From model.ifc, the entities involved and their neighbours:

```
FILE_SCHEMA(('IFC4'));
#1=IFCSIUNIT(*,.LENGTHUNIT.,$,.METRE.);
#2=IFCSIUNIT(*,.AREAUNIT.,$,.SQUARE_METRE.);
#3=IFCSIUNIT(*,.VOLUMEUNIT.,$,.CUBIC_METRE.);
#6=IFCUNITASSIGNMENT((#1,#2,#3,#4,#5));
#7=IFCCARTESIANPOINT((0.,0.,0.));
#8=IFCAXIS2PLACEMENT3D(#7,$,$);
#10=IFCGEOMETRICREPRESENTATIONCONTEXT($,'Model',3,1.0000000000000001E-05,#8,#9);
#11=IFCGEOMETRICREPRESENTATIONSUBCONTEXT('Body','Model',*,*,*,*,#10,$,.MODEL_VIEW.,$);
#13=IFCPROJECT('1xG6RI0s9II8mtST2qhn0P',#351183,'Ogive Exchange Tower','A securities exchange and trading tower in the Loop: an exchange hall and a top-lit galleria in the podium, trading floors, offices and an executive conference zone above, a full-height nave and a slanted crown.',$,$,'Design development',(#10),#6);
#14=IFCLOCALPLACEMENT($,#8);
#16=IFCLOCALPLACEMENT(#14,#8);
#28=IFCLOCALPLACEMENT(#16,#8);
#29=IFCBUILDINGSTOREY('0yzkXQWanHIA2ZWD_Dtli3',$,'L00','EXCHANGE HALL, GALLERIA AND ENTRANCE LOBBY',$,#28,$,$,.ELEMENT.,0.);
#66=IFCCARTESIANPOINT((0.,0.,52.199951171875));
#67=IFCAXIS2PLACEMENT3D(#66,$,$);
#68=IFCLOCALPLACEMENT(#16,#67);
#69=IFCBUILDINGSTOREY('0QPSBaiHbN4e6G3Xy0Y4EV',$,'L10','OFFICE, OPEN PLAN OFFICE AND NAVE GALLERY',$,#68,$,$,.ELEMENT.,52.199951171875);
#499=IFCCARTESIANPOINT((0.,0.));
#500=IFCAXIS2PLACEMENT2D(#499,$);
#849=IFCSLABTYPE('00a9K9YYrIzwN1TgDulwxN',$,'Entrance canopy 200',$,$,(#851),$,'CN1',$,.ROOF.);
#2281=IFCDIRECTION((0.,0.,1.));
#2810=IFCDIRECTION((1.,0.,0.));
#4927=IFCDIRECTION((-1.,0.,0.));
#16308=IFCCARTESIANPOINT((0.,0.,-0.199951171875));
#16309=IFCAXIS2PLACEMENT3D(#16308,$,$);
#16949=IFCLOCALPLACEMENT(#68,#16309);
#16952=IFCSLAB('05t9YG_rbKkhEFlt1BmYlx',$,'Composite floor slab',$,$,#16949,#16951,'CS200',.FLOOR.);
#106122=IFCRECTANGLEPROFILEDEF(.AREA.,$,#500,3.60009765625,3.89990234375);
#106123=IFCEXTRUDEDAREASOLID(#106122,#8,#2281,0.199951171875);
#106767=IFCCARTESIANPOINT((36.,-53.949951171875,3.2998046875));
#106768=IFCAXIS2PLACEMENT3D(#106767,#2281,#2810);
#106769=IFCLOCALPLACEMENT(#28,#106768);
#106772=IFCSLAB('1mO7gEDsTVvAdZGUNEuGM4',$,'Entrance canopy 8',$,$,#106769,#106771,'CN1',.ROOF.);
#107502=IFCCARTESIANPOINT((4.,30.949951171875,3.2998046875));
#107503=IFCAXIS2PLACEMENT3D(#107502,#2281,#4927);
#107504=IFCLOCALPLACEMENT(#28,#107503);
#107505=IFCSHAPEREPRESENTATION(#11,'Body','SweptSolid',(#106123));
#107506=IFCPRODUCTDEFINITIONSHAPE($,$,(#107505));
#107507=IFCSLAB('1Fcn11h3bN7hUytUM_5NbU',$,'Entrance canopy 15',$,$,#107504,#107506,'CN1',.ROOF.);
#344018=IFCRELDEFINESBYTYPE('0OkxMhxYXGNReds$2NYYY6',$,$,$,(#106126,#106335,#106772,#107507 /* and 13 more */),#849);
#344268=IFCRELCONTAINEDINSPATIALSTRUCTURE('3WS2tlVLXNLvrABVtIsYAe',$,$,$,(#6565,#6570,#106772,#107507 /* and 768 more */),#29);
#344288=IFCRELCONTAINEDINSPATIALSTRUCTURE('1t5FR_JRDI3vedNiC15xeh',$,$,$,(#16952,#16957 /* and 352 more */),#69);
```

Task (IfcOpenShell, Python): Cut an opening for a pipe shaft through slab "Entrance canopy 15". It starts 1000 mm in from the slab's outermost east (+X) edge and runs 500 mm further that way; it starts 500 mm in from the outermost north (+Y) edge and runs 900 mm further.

```python
import numpy as np
import ifcopenshell
import ifcopenshell.api.feature
import ifcopenshell.api.geometry
import ifcopenshell.api.root
import ifcopenshell.geom
import ifcopenshell.util.placement
import ifcopenshell.util.representation
import ifcopenshell.util.shape
import ifcopenshell.util.unit

model = ifcopenshell.open("model.ifc")
unit_scale = ifcopenshell.util.unit.calculate_unit_scale(model)
settings = ifcopenshell.geom.settings()


def volume(element):
    """Net volume in cubic metres, openings subtracted."""
    shape = ifcopenshell.geom.create_shape(settings, element)
    return ifcopenshell.util.shape.get_volume(shape.geometry)


slab = model.by_guid("1Fcn11h3bN7hUytUM_5NbU")
before = volume(slab)

# Extent in the slab's own axes, in metres. The edges named are its -X and -Y sides.
slab_shape = ifcopenshell.geom.create_shape(settings, slab)
vertices = ifcopenshell.util.shape.get_vertices(slab_shape.geometry)
x_min, y_min, bottom = vertices.min(axis=0)
top = vertices[:, 2].max()

opening = ifcopenshell.api.root.create_entity(model, ifc_class="IfcOpeningElement", name="Pipe shaft opening", predefined_type="OPENING")
context = ifcopenshell.util.representation.get_context(model, "Model", "Body", "MODEL_VIEW")
width, depth = 0.5, 0.9
outline = [(0.0, 0.0), (width, 0.0), (width, depth), (0.0, depth), (0.0, 0.0)]
# Overshoot both faces by 50 mm so the cut is clean.
shape = ifcopenshell.api.geometry.add_slab_representation(
    model, context=context, depth=top - bottom + 0.1, polyline=outline
)
ifcopenshell.api.geometry.assign_representation(model, product=opening, representation=shape)

matrix = ifcopenshell.util.placement.get_local_placement(slab.ObjectPlacement)
matrix[:, 3] = matrix @ np.append(np.array([x_min + 1, y_min + 0.5, bottom - 0.05]) / unit_scale, 1.0)
ifcopenshell.api.geometry.edit_object_placement(model, product=opening, matrix=matrix, is_si=False)
ifcopenshell.api.feature.add_feature(model, feature=opening, element=slab)

after = volume(slab)

print(f"slab volume {before:.3f} -> {after:.3f} m3")

model.write("model_v2.ifc")
```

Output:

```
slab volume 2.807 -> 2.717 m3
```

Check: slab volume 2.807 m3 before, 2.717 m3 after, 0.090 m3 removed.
